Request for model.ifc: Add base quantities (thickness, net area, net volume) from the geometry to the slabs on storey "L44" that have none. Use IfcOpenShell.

First a look at what the model holds.

```python
import ifcopenshell
import ifcopenshell.util.element
import ifcopenshell.util.unit

model = ifcopenshell.open("model.ifc")
print(model.schema)
for unit_type in ("LENGTHUNIT", "AREAUNIT", "VOLUMEUNIT"):
    print(unit_type, ifcopenshell.util.unit.calculate_unit_scale(model, unit_type))
storey = next(s for s in model.by_type("IfcBuildingStorey") if s.Name == "L44")
slabs = [e for e in ifcopenshell.util.element.get_decomposition(storey) if e.is_a("IfcSlab")]
for e in sorted(slabs, key=lambda e: e.id()):
    print(e.id(), e.is_a(), e.Name, list(ifcopenshell.util.element.get_psets(e, qtos_only=True)), sep=" | ")
```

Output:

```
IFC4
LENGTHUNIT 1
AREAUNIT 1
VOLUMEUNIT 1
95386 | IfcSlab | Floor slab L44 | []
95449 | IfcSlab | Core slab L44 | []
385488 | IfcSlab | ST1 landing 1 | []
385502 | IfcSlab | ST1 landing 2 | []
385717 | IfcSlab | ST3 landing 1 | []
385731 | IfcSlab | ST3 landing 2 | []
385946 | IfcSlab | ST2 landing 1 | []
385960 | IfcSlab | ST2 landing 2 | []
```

```python
import ifcopenshell
import ifcopenshell.api.pset
import ifcopenshell.geom
import ifcopenshell.util.element
import ifcopenshell.util.shape
import ifcopenshell.util.unit

model = ifcopenshell.open("model.ifc")
unit_scale = ifcopenshell.util.unit.calculate_unit_scale(model)
area_scale = ifcopenshell.util.unit.calculate_unit_scale(model, "AREAUNIT")
volume_scale = ifcopenshell.util.unit.calculate_unit_scale(model, "VOLUMEUNIT")
settings = ifcopenshell.geom.settings()

storey = next(s for s in model.by_type("IfcBuildingStorey") if s.Name == "L44")
slabs = [e for e in ifcopenshell.util.element.get_decomposition(storey) if e.is_a("IfcSlab")]

for e in sorted(slabs, key=lambda e: e.id()):
    if ifcopenshell.util.element.get_psets(e, qtos_only=True, should_inherit=False):
        continue
    # Geometry comes back in metres, in the element's own axes.
    shape = ifcopenshell.geom.create_shape(settings, e)
    values = {
        "Width": ifcopenshell.util.shape.get_z(shape.geometry) / unit_scale,
        "NetArea": ifcopenshell.util.shape.get_footprint_area(shape.geometry) / area_scale,
        "NetVolume": ifcopenshell.util.shape.get_volume(shape.geometry) / volume_scale,
    }
    qto = ifcopenshell.api.pset.add_qto(model, product=e, name="Qto_SlabBaseQuantities")
    ifcopenshell.api.pset.edit_qto(model, qto=qto, properties=values)
    print(e.id(), {k: round(v, 3) for k, v in values.items()})

model.write("model-out.ifc")
```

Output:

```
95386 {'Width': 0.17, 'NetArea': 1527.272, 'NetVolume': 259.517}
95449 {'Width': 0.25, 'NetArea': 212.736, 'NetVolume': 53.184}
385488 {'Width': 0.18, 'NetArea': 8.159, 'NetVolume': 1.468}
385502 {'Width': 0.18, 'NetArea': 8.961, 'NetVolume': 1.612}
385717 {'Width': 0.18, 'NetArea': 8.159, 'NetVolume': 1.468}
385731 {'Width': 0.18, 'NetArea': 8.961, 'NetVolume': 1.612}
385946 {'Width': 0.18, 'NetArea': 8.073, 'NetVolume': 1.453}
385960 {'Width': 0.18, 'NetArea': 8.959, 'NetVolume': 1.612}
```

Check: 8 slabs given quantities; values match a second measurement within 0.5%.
